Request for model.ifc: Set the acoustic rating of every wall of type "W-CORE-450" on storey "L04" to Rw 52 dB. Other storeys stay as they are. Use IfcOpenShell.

First a look at what the model holds.

```python
import ifcopenshell
import ifcopenshell.util.element

model = ifcopenshell.open("model.ifc")
print(model.schema)
storey = next(s for s in model.by_type("IfcBuildingStorey") if s.Name == "L04")
walls = [e for e in ifcopenshell.util.element.get_decomposition(storey) if e.is_a("IfcWall")]
seen = {}
for e in walls:
    element_type = ifcopenshell.util.element.get_type(e)
    key = (element_type.Name if element_type != e and element_type else None, ifcopenshell.util.element.get_pset(e, "Pset_WallCommon", "AcousticRating"))
    seen[key] = seen.get(key, 0) + 1
for (name, value), count in sorted(seen.items(), key=str):
    print(count, "x", name, "|", value)
```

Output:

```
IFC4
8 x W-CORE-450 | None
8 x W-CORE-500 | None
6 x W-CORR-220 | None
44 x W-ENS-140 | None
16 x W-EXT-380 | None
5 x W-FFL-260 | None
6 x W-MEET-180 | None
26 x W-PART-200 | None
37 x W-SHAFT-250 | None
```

```python
import ifcopenshell
import ifcopenshell.api.pset
import ifcopenshell.util.element

model = ifcopenshell.open("model.ifc")

storey = next(s for s in model.by_type("IfcBuildingStorey") if s.Name == "L04")
walls = [e for e in ifcopenshell.util.element.get_decomposition(storey) if e.is_a("IfcWall")]

count = 0
for e in walls:
    element_type = ifcopenshell.util.element.get_type(e)
    if element_type in (None, e) or element_type.Name != "W-CORE-450":
        continue
    # add_pset returns the element's existing set when there is one.
    pset = ifcopenshell.api.pset.add_pset(model, product=e, name="Pset_WallCommon")
    ifcopenshell.api.pset.edit_pset(model, pset=pset, properties={"AcousticRating": "Rw 52 dB"})
    count += 1

print(count, "walls updated")

model.write("model_edited.ifc")
```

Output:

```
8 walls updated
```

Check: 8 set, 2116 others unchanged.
